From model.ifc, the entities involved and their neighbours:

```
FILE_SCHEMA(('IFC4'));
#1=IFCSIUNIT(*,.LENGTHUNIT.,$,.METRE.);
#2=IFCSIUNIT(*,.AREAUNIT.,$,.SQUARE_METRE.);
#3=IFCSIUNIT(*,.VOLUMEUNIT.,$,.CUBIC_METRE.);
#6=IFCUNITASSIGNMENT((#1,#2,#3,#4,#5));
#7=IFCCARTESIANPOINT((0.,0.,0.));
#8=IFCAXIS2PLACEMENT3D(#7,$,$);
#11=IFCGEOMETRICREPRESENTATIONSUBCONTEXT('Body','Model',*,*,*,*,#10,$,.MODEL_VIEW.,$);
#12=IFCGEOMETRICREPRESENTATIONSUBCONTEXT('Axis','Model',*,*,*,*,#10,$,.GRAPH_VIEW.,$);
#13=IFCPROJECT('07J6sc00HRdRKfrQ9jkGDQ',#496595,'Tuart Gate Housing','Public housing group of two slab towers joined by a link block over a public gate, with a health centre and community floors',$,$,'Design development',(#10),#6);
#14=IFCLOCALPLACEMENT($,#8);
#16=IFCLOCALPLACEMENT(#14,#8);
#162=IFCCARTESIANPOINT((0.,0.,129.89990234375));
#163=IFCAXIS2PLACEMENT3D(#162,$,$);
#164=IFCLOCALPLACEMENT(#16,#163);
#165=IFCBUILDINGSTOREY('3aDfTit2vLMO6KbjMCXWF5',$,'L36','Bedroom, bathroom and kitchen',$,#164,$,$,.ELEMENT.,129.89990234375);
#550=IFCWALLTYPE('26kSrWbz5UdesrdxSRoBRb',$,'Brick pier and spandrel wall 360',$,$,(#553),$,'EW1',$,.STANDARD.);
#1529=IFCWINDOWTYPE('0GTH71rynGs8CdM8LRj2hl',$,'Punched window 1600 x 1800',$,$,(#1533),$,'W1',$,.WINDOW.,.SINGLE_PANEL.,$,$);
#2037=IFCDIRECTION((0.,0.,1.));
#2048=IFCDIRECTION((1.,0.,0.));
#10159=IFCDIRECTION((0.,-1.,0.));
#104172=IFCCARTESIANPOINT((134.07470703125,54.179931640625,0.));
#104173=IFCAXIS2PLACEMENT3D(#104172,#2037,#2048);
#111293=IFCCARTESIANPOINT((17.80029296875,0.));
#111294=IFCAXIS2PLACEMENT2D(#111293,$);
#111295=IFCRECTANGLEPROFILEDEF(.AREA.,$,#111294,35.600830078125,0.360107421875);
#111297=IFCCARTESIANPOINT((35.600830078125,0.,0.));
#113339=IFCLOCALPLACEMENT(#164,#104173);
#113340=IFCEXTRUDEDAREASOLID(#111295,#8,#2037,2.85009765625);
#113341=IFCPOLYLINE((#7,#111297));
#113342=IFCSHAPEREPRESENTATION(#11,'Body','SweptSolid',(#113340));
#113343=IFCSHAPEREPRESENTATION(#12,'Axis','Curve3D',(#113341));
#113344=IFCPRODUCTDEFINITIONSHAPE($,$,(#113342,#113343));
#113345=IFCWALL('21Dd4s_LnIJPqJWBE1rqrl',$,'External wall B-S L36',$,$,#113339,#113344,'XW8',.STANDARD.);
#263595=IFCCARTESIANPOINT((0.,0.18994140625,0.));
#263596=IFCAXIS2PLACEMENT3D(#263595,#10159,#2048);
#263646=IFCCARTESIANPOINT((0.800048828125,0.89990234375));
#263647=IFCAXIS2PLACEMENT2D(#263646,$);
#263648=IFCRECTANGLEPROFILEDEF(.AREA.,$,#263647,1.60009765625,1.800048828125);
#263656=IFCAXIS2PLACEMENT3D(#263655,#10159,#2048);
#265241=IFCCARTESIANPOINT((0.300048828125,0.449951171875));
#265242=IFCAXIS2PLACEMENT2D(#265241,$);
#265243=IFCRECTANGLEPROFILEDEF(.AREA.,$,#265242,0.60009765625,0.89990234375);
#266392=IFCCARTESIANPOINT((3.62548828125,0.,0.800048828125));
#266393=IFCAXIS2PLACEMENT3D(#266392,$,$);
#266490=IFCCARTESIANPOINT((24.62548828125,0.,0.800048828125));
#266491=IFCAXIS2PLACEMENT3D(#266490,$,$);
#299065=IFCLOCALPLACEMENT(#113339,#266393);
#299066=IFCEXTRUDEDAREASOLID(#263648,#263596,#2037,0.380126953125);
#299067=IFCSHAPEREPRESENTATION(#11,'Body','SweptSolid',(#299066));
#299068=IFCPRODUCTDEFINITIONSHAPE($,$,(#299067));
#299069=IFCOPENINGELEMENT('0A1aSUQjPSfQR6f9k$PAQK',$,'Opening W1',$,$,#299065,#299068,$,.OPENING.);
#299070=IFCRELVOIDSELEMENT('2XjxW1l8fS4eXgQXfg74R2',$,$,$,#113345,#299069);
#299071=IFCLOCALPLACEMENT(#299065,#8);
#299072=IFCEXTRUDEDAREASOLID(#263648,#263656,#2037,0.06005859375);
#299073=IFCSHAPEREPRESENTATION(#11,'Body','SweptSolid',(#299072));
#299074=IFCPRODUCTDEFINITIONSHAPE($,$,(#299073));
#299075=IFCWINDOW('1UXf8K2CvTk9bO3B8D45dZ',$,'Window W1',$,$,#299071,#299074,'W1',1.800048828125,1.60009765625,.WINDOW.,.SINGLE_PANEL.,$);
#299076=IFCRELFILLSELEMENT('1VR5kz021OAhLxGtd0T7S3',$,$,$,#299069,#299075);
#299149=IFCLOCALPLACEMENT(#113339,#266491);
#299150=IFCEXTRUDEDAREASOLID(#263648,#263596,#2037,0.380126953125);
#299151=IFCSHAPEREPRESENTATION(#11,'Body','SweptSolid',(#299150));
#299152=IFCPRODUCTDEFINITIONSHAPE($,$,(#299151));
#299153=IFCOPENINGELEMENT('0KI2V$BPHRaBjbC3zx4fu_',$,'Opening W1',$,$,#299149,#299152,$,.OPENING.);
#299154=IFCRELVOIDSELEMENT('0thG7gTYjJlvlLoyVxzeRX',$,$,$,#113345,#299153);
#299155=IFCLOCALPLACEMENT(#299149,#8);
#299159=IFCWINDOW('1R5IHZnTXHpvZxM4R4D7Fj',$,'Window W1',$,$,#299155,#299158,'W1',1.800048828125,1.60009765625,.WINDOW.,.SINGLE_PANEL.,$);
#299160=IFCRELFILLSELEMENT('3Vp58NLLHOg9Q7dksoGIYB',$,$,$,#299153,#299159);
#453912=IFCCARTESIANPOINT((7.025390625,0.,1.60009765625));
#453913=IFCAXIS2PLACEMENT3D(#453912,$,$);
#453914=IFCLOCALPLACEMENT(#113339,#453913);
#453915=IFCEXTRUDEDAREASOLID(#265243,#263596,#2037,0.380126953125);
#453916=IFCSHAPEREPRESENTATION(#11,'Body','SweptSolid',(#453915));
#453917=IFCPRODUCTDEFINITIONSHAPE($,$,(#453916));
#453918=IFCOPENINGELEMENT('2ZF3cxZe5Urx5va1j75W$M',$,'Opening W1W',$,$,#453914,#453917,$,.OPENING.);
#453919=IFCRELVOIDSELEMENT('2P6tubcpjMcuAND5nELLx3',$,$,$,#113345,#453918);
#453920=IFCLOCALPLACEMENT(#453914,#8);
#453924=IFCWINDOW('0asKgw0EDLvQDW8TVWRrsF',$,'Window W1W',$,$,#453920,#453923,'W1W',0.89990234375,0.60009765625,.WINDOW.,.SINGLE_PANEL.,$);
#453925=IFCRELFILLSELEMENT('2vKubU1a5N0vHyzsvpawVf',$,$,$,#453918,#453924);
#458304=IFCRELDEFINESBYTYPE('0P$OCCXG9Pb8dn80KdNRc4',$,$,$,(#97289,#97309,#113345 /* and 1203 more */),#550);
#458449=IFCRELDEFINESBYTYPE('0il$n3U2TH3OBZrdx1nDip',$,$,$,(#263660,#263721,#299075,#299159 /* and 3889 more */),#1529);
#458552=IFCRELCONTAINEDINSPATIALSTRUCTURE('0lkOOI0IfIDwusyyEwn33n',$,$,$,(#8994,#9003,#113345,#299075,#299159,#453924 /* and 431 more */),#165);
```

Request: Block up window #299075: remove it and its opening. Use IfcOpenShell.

```python
import ifcopenshell
import ifcopenshell.api.feature
import ifcopenshell.api.root
import ifcopenshell.geom
import ifcopenshell.util.shape

model = ifcopenshell.open("model.ifc")
settings = ifcopenshell.geom.settings()


def volume(element):
    """Net volume in cubic metres, openings subtracted."""
    shape = ifcopenshell.geom.create_shape(settings, element)
    return ifcopenshell.util.shape.get_volume(shape.geometry)


window = model.by_guid("1UXf8K2CvTk9bO3B8D45dZ")
opening = window.FillsVoids[0].RelatingOpeningElement
wall = opening.VoidsElements[0].RelatingBuildingElement
before = volume(wall)

ifcopenshell.api.root.remove_product(model, product=window)
ifcopenshell.api.feature.remove_feature(model, feature=opening)

after = volume(wall)

print(f"wall volume {before:.3f} -> {after:.3f} m3")

model.write("model_updated.ifc")
```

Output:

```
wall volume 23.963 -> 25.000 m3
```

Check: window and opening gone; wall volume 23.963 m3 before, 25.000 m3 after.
